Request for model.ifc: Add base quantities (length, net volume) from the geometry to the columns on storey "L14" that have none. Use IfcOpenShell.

First a look at what the model holds.

```python
import ifcopenshell
import ifcopenshell.util.element
import ifcopenshell.util.unit

model = ifcopenshell.open("model.ifc")
print(model.schema)
for unit_type in ("LENGTHUNIT", "AREAUNIT", "VOLUMEUNIT"):
    print(unit_type, ifcopenshell.util.unit.calculate_unit_scale(model, unit_type))
storey = next(s for s in model.by_type("IfcBuildingStorey") if s.Name == "L14")
columns = [e for e in ifcopenshell.util.element.get_decomposition(storey) if e.is_a("IfcColumn")]
for e in sorted(columns, key=lambda e: e.id()):
    print(e.id(), e.is_a(), e.Name, list(ifcopenshell.util.element.get_psets(e, qtos_only=True)), sep=" | ")
```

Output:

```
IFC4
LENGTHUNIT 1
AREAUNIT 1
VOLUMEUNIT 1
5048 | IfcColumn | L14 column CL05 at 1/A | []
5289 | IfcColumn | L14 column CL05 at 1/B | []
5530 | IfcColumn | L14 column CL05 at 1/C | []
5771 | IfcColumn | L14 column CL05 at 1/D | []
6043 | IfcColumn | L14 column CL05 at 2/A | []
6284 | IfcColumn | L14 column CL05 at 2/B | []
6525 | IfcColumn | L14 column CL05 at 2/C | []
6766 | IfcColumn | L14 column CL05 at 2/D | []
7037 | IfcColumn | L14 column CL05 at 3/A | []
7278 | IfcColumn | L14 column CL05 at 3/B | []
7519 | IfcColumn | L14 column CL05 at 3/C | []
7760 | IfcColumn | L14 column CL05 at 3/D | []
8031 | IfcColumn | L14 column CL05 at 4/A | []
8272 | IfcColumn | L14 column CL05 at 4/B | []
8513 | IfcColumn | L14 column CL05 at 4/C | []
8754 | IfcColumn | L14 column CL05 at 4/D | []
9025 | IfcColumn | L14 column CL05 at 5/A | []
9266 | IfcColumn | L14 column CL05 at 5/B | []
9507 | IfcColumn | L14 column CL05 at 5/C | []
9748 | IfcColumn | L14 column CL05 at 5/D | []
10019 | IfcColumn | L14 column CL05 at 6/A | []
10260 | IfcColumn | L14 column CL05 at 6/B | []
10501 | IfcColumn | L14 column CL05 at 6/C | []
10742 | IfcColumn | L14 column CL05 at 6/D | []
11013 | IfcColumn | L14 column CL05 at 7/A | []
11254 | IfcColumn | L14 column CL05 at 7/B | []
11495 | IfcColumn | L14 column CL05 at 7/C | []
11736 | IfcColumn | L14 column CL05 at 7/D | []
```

```python
import ifcopenshell
import ifcopenshell.api.pset
import ifcopenshell.geom
import ifcopenshell.util.element
import ifcopenshell.util.shape
import ifcopenshell.util.unit

model = ifcopenshell.open("model.ifc")
unit_scale = ifcopenshell.util.unit.calculate_unit_scale(model)
volume_scale = ifcopenshell.util.unit.calculate_unit_scale(model, "VOLUMEUNIT")
settings = ifcopenshell.geom.settings()

storey = next(s for s in model.by_type("IfcBuildingStorey") if s.Name == "L14")
columns = [e for e in ifcopenshell.util.element.get_decomposition(storey) if e.is_a("IfcColumn")]

for e in sorted(columns, key=lambda e: e.id()):
    if ifcopenshell.util.element.get_psets(e, qtos_only=True, should_inherit=False):
        continue
    # Geometry comes back in metres, in the element's own axes.
    shape = ifcopenshell.geom.create_shape(settings, e)
    values = {
        "Length": ifcopenshell.util.shape.get_z(shape.geometry) / unit_scale,
        "NetVolume": ifcopenshell.util.shape.get_volume(shape.geometry) / volume_scale,
    }
    qto = ifcopenshell.api.pset.add_qto(model, product=e, name="Qto_ColumnBaseQuantities")
    ifcopenshell.api.pset.edit_qto(model, qto=qto, properties=values)
    print(e.id(), {k: round(v, 3) for k, v in values.items()})

model.write("model_v2.ifc")
```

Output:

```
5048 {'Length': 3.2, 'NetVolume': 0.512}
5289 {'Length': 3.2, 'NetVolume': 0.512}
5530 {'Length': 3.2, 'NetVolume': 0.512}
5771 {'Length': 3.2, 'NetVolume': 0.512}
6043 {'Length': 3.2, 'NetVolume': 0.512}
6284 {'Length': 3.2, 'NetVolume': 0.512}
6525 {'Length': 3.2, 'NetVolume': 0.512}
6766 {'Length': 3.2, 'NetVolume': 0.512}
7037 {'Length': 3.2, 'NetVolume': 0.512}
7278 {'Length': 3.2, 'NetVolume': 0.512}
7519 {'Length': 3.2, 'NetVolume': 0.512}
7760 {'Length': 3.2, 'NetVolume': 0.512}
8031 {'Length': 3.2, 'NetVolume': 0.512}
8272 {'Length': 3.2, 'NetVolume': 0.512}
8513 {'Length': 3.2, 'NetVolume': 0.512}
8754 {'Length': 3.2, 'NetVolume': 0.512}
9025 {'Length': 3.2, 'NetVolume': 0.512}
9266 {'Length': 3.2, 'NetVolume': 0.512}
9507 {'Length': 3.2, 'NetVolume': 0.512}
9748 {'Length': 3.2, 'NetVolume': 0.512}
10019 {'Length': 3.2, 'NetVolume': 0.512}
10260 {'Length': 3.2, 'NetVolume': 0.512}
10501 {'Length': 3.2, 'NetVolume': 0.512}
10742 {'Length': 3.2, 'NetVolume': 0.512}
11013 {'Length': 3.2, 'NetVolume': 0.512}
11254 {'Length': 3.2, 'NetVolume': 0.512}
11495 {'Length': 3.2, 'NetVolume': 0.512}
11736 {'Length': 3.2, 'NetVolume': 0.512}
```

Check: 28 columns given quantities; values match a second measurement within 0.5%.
